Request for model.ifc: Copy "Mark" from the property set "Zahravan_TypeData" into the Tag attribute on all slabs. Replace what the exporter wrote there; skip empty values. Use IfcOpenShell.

First a look at what the model holds.

```python
import ifcopenshell
import ifcopenshell.util.element

model = ifcopenshell.open("model.ifc")
print(model.schema)
slabs = model.by_type("IfcSlab")
print(len(slabs), "slabs")
for e in slabs[:8]:
    source = ifcopenshell.util.element.get_pset(e, "Zahravan_TypeData", "Mark")
    target = e.Tag
    print(e.id(), repr(source), repr(target), sep=" | ")
```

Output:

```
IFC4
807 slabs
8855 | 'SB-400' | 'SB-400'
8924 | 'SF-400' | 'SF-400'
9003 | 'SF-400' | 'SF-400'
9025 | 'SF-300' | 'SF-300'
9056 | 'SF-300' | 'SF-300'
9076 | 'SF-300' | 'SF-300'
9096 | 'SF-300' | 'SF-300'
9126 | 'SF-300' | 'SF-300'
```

```python
import ifcopenshell
import ifcopenshell.util.element

model = ifcopenshell.open("model.ifc")

count = 0
for e in model.by_type("IfcSlab"):
    value = ifcopenshell.util.element.get_pset(e, "Zahravan_TypeData", "Mark")
    current = e.Tag
    if not value or not value.strip() or current == value:
        continue
    e.Tag = value
    count += 1

print(count, "slabs updated")

model.write("model_v2.ifc")
```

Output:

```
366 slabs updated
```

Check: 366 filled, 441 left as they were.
